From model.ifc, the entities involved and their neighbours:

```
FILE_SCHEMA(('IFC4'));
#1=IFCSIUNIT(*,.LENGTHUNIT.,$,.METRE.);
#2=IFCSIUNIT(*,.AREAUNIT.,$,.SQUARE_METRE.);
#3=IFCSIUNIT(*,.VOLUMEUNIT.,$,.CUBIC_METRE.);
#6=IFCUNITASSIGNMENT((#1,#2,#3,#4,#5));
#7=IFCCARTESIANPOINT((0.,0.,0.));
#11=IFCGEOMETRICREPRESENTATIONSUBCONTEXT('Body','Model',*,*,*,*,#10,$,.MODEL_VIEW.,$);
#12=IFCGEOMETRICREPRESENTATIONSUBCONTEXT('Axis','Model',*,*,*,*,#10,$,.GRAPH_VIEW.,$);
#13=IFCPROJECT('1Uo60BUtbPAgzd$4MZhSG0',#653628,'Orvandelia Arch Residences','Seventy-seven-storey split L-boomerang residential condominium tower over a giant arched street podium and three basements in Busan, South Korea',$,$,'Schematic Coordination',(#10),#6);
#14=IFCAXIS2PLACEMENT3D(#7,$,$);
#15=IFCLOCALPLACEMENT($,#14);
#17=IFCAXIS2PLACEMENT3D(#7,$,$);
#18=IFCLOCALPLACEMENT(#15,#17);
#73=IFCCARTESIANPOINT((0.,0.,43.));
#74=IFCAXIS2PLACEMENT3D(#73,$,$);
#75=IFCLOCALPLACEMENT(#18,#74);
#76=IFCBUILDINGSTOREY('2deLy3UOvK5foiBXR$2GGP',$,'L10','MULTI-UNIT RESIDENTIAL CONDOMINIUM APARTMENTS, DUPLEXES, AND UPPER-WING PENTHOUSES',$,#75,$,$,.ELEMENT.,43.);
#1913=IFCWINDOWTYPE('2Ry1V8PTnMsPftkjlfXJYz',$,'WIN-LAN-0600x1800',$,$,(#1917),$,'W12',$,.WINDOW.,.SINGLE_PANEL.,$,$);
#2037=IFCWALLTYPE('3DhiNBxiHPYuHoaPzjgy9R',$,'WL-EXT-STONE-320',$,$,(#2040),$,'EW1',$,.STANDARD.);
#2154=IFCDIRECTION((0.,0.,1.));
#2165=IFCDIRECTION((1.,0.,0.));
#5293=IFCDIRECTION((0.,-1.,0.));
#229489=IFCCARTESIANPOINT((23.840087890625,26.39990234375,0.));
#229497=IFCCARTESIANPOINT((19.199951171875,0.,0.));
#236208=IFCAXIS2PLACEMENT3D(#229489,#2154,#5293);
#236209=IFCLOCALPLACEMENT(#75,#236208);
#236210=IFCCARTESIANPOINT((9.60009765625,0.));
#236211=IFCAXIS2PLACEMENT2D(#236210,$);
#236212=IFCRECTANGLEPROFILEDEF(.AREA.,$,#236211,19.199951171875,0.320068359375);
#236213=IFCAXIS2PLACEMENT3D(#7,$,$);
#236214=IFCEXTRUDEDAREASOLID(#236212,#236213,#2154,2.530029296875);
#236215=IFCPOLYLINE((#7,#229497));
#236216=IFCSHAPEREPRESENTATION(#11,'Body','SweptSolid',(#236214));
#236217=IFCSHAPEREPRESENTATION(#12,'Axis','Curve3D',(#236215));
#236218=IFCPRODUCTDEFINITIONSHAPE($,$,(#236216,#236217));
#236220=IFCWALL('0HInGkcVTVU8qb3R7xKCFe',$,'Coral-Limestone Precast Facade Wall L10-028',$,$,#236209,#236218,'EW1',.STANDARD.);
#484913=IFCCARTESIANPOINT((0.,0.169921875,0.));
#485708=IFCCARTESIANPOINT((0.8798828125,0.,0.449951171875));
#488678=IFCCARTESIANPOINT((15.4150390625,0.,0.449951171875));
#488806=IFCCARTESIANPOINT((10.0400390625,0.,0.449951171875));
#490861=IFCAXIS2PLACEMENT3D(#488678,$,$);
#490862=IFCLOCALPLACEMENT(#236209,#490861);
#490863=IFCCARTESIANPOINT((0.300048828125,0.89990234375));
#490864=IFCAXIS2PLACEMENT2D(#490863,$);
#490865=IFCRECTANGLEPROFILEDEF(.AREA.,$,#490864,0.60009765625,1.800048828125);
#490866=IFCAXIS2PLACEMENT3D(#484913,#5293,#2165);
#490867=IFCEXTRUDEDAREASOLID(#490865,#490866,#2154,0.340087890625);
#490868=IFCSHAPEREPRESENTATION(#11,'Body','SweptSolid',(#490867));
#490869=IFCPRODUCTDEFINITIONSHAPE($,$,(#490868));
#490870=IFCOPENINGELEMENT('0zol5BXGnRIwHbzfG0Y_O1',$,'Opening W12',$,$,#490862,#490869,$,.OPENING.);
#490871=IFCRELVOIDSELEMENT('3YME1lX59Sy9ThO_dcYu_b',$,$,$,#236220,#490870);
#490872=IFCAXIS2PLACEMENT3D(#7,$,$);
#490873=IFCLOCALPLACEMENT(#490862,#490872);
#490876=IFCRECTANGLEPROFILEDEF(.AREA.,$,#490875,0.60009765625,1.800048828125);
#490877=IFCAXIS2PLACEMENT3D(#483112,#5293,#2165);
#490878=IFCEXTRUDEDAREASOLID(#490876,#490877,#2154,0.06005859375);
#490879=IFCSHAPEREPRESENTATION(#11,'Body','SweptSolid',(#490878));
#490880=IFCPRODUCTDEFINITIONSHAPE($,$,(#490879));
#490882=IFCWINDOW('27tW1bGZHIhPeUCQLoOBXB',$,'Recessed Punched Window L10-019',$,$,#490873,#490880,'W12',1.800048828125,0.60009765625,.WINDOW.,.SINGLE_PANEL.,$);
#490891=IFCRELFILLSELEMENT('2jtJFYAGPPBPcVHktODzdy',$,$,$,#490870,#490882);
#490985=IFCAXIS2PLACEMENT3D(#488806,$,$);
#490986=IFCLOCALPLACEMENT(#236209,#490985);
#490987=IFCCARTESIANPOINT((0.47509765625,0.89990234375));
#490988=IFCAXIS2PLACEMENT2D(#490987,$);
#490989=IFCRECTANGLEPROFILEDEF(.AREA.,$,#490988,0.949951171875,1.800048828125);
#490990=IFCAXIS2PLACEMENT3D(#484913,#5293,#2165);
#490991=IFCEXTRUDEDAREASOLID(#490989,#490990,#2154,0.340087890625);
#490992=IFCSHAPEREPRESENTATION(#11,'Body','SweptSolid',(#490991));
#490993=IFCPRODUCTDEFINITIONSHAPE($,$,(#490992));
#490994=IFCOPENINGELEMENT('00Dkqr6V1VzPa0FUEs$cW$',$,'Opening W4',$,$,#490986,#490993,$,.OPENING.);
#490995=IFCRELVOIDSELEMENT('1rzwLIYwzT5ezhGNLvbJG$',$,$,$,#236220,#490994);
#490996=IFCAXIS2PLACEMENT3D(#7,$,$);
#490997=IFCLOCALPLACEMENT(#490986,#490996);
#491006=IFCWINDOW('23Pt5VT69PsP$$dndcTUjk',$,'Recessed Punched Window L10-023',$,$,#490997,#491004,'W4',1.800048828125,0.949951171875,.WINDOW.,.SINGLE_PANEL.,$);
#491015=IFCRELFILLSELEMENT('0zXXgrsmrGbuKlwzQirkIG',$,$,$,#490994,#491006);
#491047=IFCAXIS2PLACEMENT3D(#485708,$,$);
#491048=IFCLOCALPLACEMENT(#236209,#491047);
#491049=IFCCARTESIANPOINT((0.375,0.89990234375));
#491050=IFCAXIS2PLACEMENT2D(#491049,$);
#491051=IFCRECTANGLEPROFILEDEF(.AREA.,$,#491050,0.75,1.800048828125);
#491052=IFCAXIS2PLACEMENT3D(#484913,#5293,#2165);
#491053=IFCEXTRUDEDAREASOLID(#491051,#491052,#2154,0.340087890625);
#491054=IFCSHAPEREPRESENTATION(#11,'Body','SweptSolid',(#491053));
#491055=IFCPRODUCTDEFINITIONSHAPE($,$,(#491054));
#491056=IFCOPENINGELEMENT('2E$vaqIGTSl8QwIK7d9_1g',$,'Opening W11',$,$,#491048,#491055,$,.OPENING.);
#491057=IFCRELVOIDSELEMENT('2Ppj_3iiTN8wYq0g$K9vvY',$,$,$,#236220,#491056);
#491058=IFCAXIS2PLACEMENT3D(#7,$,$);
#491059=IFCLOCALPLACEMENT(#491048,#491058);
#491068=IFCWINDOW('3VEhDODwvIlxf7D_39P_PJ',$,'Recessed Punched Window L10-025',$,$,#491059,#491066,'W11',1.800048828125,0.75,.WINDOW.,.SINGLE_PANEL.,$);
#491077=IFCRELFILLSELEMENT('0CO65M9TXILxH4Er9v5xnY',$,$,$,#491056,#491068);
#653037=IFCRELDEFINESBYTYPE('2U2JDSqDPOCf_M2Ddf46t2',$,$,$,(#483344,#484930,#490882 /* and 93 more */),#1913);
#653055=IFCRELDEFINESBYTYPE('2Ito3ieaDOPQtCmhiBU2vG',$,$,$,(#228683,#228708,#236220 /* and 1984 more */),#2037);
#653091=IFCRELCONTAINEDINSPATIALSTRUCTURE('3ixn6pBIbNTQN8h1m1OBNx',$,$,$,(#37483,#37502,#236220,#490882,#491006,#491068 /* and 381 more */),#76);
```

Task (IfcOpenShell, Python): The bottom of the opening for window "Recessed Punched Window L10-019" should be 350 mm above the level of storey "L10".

```python
import numpy as np
import ifcopenshell
import ifcopenshell.api.geometry
import ifcopenshell.geom
import ifcopenshell.util.element
import ifcopenshell.util.placement
import ifcopenshell.util.shape
import ifcopenshell.util.unit

model = ifcopenshell.open("model.ifc")
unit_scale = ifcopenshell.util.unit.calculate_unit_scale(model)

window = model.by_guid("27tW1bGZHIhPeUCQLoOBXB")
opening = window.FillsVoids[0].RelatingOpeningElement
storey = ifcopenshell.util.element.get_container(window, ifc_class="IfcBuildingStorey")
level = ifcopenshell.util.placement.get_local_placement(storey.ObjectPlacement)[2, 3]

# The opening's origin need not be at the sill, so measure its lowest point.
shape = ifcopenshell.geom.create_shape(ifcopenshell.geom.settings(), opening)
bottom = ifcopenshell.util.shape.get_shape_bottom_elevation(shape, shape.geometry) / unit_scale
dz = level + 0.35 - bottom

shift = np.array([0.0, 0.0, dz])
# The window is placed relative to its opening, so it follows when the opening moves.
matrix = ifcopenshell.util.placement.get_local_placement(opening.ObjectPlacement)
matrix[:3, 3] += shift
ifcopenshell.api.geometry.edit_object_placement(
    model, product=opening, matrix=matrix, is_si=False, should_transform_children=True
)

print(f"moved by {dz * unit_scale:+.3f} m")

model.write("model_edited.ifc")
```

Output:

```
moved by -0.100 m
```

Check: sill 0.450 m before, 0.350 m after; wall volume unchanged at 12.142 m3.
